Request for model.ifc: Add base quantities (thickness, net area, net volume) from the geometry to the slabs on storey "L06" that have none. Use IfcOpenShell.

First a look at what the model holds.

```python
import ifcopenshell
import ifcopenshell.util.element
import ifcopenshell.util.unit

model = ifcopenshell.open("model.ifc")
print(model.schema)
for unit_type in ("LENGTHUNIT", "AREAUNIT", "VOLUMEUNIT"):
    print(unit_type, ifcopenshell.util.unit.calculate_unit_scale(model, unit_type))
storey = next(s for s in model.by_type("IfcBuildingStorey") if s.Name == "L06")
slabs = [e for e in ifcopenshell.util.element.get_decomposition(storey) if e.is_a("IfcSlab")]
for e in sorted(slabs, key=lambda e: e.id()):
    print(e.id(), e.is_a(), e.Name, list(ifcopenshell.util.element.get_psets(e, qtos_only=True)), sep=" | ")
```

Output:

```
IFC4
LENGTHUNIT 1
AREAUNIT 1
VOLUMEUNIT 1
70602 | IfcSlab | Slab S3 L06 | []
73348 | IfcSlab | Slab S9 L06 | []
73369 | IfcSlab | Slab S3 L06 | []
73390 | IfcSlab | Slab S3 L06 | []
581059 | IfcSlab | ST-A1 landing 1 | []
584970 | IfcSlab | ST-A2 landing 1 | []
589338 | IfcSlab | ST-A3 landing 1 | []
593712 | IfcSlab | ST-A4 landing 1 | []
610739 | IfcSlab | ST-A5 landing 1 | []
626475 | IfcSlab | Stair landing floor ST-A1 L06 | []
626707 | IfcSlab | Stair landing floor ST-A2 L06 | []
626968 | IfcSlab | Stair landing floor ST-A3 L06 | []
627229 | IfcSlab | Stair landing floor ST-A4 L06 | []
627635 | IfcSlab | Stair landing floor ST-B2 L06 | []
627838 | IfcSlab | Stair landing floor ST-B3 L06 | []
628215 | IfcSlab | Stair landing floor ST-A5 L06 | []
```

```python
import ifcopenshell
import ifcopenshell.api.pset
import ifcopenshell.geom
import ifcopenshell.util.element
import ifcopenshell.util.shape
import ifcopenshell.util.unit

model = ifcopenshell.open("model.ifc")
unit_scale = ifcopenshell.util.unit.calculate_unit_scale(model)
area_scale = ifcopenshell.util.unit.calculate_unit_scale(model, "AREAUNIT")
volume_scale = ifcopenshell.util.unit.calculate_unit_scale(model, "VOLUMEUNIT")
settings = ifcopenshell.geom.settings()

storey = next(s for s in model.by_type("IfcBuildingStorey") if s.Name == "L06")
slabs = [e for e in ifcopenshell.util.element.get_decomposition(storey) if e.is_a("IfcSlab")]

for e in sorted(slabs, key=lambda e: e.id()):
    if ifcopenshell.util.element.get_psets(e, qtos_only=True, should_inherit=False):
        continue
    # Geometry comes back in metres, in the element's own axes.
    shape = ifcopenshell.geom.create_shape(settings, e)
    values = {
        "Width": ifcopenshell.util.shape.get_z(shape.geometry) / unit_scale,
        "NetArea": ifcopenshell.util.shape.get_footprint_area(shape.geometry) / area_scale,
        "NetVolume": ifcopenshell.util.shape.get_volume(shape.geometry) / volume_scale,
    }
    qto = ifcopenshell.api.pset.add_qto(model, product=e, name="Qto_SlabBaseQuantities")
    ifcopenshell.api.pset.edit_qto(model, qto=qto, properties=values)
    print(e.id(), {k: round(v, 3) for k, v in values.items()})

model.write("model_v2.ifc")
```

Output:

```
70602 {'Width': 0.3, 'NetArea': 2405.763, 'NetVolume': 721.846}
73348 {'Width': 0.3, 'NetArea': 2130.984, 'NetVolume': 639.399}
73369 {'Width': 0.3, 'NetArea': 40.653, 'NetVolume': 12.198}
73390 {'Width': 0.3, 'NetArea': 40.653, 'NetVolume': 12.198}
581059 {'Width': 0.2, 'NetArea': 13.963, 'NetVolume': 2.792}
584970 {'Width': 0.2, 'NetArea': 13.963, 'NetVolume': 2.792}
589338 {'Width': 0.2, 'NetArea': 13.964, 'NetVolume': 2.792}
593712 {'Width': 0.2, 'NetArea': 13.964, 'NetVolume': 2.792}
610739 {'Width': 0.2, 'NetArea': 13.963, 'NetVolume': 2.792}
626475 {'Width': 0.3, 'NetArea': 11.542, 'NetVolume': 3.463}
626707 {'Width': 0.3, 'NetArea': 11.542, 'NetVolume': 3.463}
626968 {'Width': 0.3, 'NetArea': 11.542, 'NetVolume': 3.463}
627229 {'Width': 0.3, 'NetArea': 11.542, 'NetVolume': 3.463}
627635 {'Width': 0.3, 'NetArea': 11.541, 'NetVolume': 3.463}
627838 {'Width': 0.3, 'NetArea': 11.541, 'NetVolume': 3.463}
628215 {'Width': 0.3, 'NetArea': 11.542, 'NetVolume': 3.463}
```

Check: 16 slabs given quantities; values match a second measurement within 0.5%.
